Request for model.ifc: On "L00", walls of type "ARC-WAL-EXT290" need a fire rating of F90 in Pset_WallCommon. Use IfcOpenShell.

First a look at what the model holds.

```python
import ifcopenshell
import ifcopenshell.util.element

model = ifcopenshell.open("model.ifc")
print(model.schema)
storey = next(s for s in model.by_type("IfcBuildingStorey") if s.Name == "L00")
walls = [e for e in ifcopenshell.util.element.get_decomposition(storey) if e.is_a("IfcWall")]
seen = {}
for e in walls:
    element_type = ifcopenshell.util.element.get_type(e)
    key = (element_type.Name if element_type != e and element_type else None, ifcopenshell.util.element.get_pset(e, "Pset_WallCommon", "FireRating"))
    seen[key] = seen.get(key, 0) + 1
for (name, value), count in sorted(seen.items(), key=str):
    print(count, "x", name, "|", value)
```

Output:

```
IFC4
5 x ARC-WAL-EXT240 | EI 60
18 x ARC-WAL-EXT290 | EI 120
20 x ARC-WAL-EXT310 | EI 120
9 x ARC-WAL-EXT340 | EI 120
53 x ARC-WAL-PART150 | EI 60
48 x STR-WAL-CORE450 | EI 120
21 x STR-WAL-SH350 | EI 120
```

```python
import ifcopenshell
import ifcopenshell.api.pset
import ifcopenshell.util.element

model = ifcopenshell.open("model.ifc")

storey = next(s for s in model.by_type("IfcBuildingStorey") if s.Name == "L00")
walls = [e for e in ifcopenshell.util.element.get_decomposition(storey) if e.is_a("IfcWall")]

count = 0
for e in walls:
    element_type = ifcopenshell.util.element.get_type(e)
    if element_type in (None, e) or element_type.Name != "ARC-WAL-EXT290":
        continue
    # add_pset returns the element's existing set when there is one.
    pset = ifcopenshell.api.pset.add_pset(model, product=e, name="Pset_WallCommon")
    ifcopenshell.api.pset.edit_pset(model, pset=pset, properties={"FireRating": "F90"})
    count += 1

print(count, "walls updated")

model.write("model_rev.ifc")
```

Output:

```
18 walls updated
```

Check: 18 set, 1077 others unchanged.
